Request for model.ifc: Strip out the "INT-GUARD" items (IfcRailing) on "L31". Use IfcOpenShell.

First a look at what the model holds.

```python
import ifcopenshell
import ifcopenshell.util.element

model = ifcopenshell.open("model.ifc")
print(model.schema)
storey = next(s for s in model.by_type("IfcBuildingStorey") if s.Name == "L31")
railings = [e for e in ifcopenshell.util.element.get_decomposition(storey) if e.is_a("IfcRailing")]
seen = {}
for e in railings:
    element_type = ifcopenshell.util.element.get_type(e)
    name = element_type.Name if element_type not in (None, e) else None
    seen[name] = seen.get(name, 0) + 1
for name, count in sorted(seen.items(), key=str):
    print(count, "x", name)
```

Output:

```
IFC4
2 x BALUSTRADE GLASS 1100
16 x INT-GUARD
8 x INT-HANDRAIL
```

```python
import ifcopenshell
import ifcopenshell.api.root
import ifcopenshell.util.element

model = ifcopenshell.open("model.ifc")

storey = next(s for s in model.by_type("IfcBuildingStorey") if s.Name == "L31")
railings = [e for e in ifcopenshell.util.element.get_decomposition(storey) if e.is_a("IfcRailing")]
targets = [e for e in railings if (t := ifcopenshell.util.element.get_type(e)) not in (None, e) and t.Name == "INT-GUARD"]

for e in targets:
    ifcopenshell.api.root.remove_product(model, product=e)
print(len(targets), "removed")

model.write("model_edited.ifc")
```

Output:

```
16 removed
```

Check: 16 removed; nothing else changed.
